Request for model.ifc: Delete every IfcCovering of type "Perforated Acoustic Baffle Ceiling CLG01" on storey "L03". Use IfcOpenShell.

First a look at what the model holds.

```python
import ifcopenshell
import ifcopenshell.util.element

model = ifcopenshell.open("model.ifc")
print(model.schema)
storey = next(s for s in model.by_type("IfcBuildingStorey") if s.Name == "L03")
coverings = [e for e in ifcopenshell.util.element.get_decomposition(storey) if e.is_a("IfcCovering")]
seen = {}
for e in coverings:
    element_type = ifcopenshell.util.element.get_type(e)
    name = element_type.Name if element_type not in (None, e) else None
    seen[name] = seen.get(name, 0) + 1
for name, count in sorted(seen.items(), key=str):
    print(count, "x", name)
```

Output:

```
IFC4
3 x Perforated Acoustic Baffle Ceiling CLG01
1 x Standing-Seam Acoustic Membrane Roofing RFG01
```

```python
import ifcopenshell
import ifcopenshell.api.root
import ifcopenshell.util.element

model = ifcopenshell.open("model.ifc")

storey = next(s for s in model.by_type("IfcBuildingStorey") if s.Name == "L03")
coverings = [e for e in ifcopenshell.util.element.get_decomposition(storey) if e.is_a("IfcCovering")]
targets = [e for e in coverings if (t := ifcopenshell.util.element.get_type(e)) not in (None, e) and t.Name == "Perforated Acoustic Baffle Ceiling CLG01"]

for e in targets:
    ifcopenshell.api.root.remove_product(model, product=e)
print(len(targets), "removed")

model.write("model-out.ifc")
```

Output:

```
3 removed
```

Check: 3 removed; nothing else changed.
